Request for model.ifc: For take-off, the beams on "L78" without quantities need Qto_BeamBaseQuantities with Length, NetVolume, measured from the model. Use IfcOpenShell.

First a look at what the model holds.

```python
import ifcopenshell
import ifcopenshell.util.element
import ifcopenshell.util.unit

model = ifcopenshell.open("model.ifc")
print(model.schema)
for unit_type in ("LENGTHUNIT", "AREAUNIT", "VOLUMEUNIT"):
    print(unit_type, ifcopenshell.util.unit.calculate_unit_scale(model, unit_type))
storey = next(s for s in model.by_type("IfcBuildingStorey") if s.Name == "L78")
beams = [e for e in ifcopenshell.util.element.get_decomposition(storey) if e.is_a("IfcBeam")]
for e in sorted(beams, key=lambda e: e.id()):
    print(e.id(), e.is_a(), e.Name, list(ifcopenshell.util.element.get_psets(e, qtos_only=True)), sep=" | ")
```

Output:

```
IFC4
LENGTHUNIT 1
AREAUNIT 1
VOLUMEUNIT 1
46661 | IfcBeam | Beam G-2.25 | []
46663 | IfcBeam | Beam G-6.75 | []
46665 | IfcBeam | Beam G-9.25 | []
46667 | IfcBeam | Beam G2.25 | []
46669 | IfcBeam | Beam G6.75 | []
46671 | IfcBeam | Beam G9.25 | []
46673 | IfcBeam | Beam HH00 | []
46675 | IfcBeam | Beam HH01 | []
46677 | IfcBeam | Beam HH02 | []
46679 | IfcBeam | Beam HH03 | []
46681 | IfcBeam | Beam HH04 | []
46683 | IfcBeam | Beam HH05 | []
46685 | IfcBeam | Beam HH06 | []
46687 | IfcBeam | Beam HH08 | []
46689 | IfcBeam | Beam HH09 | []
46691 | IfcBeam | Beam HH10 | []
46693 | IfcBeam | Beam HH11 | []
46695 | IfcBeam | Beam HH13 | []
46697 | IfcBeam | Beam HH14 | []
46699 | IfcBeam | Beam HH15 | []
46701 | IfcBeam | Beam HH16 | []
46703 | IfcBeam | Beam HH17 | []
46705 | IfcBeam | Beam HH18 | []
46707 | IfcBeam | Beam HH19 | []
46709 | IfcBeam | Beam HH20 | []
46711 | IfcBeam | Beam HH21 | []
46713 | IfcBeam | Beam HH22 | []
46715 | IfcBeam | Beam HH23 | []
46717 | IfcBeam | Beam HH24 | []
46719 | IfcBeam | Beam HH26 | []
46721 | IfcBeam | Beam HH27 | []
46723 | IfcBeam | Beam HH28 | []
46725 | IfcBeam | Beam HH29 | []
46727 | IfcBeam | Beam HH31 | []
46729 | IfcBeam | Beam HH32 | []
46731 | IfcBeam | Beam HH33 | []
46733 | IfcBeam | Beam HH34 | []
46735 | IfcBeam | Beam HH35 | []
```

```python
import ifcopenshell
import ifcopenshell.api.pset
import ifcopenshell.geom
import ifcopenshell.util.element
import ifcopenshell.util.shape
import ifcopenshell.util.unit

model = ifcopenshell.open("model.ifc")
unit_scale = ifcopenshell.util.unit.calculate_unit_scale(model)
volume_scale = ifcopenshell.util.unit.calculate_unit_scale(model, "VOLUMEUNIT")
settings = ifcopenshell.geom.settings()

storey = next(s for s in model.by_type("IfcBuildingStorey") if s.Name == "L78")
beams = [e for e in ifcopenshell.util.element.get_decomposition(storey) if e.is_a("IfcBeam")]

for e in sorted(beams, key=lambda e: e.id()):
    if ifcopenshell.util.element.get_psets(e, qtos_only=True, should_inherit=False):
        continue
    # Geometry comes back in metres, in the element's own axes.
    shape = ifcopenshell.geom.create_shape(settings, e)
    values = {
        "Length": ifcopenshell.util.shape.get_max_xyz(shape.geometry) / unit_scale,
        "NetVolume": ifcopenshell.util.shape.get_volume(shape.geometry) / volume_scale,
    }
    qto = ifcopenshell.api.pset.add_qto(model, product=e, name="Qto_BeamBaseQuantities")
    ifcopenshell.api.pset.edit_qto(model, qto=qto, properties=values)
    print(e.id(), {k: round(v, 3) for k, v in values.items()})

model.write("model-out.ifc")
```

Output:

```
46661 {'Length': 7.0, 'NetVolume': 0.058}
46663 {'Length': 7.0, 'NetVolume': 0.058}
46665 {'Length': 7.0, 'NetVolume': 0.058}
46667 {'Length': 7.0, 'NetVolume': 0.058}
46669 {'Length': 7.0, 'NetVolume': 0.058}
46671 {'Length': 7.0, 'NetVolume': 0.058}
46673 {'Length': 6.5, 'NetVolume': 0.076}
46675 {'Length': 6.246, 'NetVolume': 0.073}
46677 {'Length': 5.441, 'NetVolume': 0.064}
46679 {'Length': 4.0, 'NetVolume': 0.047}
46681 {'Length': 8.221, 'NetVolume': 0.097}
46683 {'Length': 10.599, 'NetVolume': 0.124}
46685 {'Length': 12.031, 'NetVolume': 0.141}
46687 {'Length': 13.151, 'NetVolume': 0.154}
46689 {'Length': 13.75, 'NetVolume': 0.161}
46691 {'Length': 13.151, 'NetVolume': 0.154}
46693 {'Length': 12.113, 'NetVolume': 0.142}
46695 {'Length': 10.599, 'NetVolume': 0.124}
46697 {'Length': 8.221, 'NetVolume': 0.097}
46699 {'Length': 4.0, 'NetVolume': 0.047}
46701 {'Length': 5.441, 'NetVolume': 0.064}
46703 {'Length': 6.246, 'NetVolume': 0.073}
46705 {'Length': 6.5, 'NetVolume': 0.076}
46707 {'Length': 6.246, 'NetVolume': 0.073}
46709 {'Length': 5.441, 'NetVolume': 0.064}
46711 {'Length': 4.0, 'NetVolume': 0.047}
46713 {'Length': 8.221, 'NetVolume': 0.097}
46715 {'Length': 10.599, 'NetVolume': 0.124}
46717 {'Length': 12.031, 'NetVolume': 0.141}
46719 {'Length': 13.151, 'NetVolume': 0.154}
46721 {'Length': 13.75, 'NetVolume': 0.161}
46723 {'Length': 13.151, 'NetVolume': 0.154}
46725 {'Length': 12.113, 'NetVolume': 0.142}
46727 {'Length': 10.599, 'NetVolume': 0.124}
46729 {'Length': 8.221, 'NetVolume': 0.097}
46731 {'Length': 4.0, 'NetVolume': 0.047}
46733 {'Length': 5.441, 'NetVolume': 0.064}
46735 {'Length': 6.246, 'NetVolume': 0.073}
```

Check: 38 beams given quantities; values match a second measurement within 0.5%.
